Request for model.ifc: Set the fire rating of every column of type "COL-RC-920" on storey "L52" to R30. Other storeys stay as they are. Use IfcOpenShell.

First a look at what the model holds.

```python
import ifcopenshell
import ifcopenshell.util.element

model = ifcopenshell.open("model.ifc")
print(model.schema)
storey = next(s for s in model.by_type("IfcBuildingStorey") if s.Name == "L52")
columns = [e for e in ifcopenshell.util.element.get_decomposition(storey) if e.is_a("IfcColumn")]
seen = {}
for e in columns:
    element_type = ifcopenshell.util.element.get_type(e)
    key = (element_type.Name if element_type != e and element_type else None, ifcopenshell.util.element.get_pset(e, "Pset_ColumnCommon", "FireRating"))
    seen[key] = seen.get(key, 0) + 1
for (name, value), count in sorted(seen.items(), key=str):
    print(count, "x", name, "|", value)
```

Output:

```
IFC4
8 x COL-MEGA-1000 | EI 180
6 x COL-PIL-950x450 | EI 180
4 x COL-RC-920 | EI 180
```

```python
import ifcopenshell
import ifcopenshell.api.pset
import ifcopenshell.util.element

model = ifcopenshell.open("model.ifc")

storey = next(s for s in model.by_type("IfcBuildingStorey") if s.Name == "L52")
columns = [e for e in ifcopenshell.util.element.get_decomposition(storey) if e.is_a("IfcColumn")]

count = 0
for e in columns:
    element_type = ifcopenshell.util.element.get_type(e)
    if element_type in (None, e) or element_type.Name != "COL-RC-920":
        continue
    found = ifcopenshell.util.element.get_pset(e, "Pset_ColumnCommon", should_inherit=False)
    if found:
        pset = model.by_id(found["id"])
        if len(ifcopenshell.util.element.get_elements_by_pset(pset)) > 1:
            pset = ifcopenshell.api.pset.unshare_pset(model, products=[e], pset=pset)[0]
    else:
        pset = ifcopenshell.api.pset.add_pset(model, product=e, name="Pset_ColumnCommon")
    ifcopenshell.api.pset.edit_pset(model, pset=pset, properties={"FireRating": "R30"})
    count += 1

print(count, "columns updated")

model.write("model-out.ifc")
```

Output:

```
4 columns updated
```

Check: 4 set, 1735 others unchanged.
